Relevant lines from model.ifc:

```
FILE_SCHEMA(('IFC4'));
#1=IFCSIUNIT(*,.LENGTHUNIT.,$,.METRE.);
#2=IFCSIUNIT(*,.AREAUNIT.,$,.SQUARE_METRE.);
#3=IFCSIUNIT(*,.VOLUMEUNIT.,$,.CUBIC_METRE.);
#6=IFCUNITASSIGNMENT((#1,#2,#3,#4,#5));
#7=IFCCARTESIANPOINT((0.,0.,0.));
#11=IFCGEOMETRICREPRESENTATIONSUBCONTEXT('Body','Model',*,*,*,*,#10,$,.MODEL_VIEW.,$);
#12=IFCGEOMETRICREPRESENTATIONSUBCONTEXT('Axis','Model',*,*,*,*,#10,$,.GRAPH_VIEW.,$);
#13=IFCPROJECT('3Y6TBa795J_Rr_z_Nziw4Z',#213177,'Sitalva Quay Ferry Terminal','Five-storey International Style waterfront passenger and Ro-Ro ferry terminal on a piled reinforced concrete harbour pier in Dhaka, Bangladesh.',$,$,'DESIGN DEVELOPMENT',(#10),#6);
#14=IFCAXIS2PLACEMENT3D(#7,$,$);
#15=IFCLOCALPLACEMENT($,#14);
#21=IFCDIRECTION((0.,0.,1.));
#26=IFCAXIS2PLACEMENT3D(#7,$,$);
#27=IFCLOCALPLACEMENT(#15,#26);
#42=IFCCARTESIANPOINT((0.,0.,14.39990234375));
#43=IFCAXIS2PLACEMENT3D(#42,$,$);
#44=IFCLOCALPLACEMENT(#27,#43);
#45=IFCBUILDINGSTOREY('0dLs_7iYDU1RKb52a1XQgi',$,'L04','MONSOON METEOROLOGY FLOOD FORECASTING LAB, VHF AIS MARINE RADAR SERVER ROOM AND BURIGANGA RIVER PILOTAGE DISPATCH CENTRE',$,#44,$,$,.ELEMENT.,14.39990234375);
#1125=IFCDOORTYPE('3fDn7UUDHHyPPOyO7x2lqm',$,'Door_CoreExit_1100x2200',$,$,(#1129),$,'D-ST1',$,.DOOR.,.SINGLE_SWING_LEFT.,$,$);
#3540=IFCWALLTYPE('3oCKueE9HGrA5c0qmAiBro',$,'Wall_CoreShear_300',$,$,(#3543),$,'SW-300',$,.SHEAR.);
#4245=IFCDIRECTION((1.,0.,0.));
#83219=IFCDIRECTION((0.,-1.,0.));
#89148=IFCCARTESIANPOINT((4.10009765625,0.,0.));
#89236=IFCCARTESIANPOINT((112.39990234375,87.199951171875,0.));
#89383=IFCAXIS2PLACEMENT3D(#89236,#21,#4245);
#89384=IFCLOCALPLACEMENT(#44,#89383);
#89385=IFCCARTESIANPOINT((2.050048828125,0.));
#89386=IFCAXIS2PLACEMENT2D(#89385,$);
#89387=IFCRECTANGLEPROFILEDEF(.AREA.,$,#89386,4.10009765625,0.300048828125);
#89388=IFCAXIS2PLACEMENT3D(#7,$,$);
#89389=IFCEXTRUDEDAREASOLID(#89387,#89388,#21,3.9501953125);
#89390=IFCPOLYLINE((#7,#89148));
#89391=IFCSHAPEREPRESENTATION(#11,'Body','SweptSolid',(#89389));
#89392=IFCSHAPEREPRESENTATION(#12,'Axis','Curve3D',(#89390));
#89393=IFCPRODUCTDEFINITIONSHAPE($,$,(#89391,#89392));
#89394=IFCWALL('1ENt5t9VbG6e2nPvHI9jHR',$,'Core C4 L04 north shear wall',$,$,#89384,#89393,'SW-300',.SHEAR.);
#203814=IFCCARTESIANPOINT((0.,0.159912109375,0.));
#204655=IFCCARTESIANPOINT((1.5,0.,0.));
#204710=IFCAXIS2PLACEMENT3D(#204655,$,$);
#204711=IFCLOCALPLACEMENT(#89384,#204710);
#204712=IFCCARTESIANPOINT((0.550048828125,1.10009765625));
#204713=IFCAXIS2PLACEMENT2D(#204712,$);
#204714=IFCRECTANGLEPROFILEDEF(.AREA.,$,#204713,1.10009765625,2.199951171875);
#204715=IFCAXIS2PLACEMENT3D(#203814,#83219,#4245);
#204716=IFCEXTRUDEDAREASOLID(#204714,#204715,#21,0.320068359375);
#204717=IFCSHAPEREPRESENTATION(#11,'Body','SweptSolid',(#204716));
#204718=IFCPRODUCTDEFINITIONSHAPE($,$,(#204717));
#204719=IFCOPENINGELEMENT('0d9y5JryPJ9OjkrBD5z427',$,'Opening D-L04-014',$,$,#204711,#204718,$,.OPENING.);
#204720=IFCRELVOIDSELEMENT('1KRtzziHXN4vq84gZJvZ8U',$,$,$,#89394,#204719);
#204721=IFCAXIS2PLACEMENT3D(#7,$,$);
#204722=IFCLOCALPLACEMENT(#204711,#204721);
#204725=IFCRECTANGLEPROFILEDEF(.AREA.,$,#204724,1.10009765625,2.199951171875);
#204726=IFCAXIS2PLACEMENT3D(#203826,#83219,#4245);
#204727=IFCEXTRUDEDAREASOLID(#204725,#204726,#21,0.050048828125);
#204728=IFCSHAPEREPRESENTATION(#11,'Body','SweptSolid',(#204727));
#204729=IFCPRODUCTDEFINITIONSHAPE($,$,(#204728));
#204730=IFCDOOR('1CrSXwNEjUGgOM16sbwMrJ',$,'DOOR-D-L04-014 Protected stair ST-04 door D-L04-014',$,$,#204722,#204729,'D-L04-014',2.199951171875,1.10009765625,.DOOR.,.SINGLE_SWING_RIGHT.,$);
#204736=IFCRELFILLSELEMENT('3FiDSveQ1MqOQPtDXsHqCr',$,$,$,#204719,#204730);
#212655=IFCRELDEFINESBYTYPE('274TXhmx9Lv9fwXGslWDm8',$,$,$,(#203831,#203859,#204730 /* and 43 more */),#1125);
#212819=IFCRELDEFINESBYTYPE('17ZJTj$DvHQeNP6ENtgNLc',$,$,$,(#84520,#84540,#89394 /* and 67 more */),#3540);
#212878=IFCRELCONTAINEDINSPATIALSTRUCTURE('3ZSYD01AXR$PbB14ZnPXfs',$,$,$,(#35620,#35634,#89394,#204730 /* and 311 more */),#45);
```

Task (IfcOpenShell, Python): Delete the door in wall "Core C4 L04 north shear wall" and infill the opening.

```python
import ifcopenshell
import ifcopenshell.api.feature
import ifcopenshell.api.root
import ifcopenshell.geom
import ifcopenshell.util.shape

model = ifcopenshell.open("model.ifc")
settings = ifcopenshell.geom.settings()


def volume(element):
    """Net volume in cubic metres, openings subtracted."""
    shape = ifcopenshell.geom.create_shape(settings, element)
    return ifcopenshell.util.shape.get_volume(shape.geometry)


door = model.by_guid("1CrSXwNEjUGgOM16sbwMrJ")
opening = door.FillsVoids[0].RelatingOpeningElement
wall = opening.VoidsElements[0].RelatingBuildingElement
before = volume(wall)

ifcopenshell.api.root.remove_product(model, product=door)
ifcopenshell.api.feature.remove_feature(model, feature=opening)

after = volume(wall)

print(f"wall volume {before:.3f} -> {after:.3f} m3")

model.write("model_updated.ifc")
```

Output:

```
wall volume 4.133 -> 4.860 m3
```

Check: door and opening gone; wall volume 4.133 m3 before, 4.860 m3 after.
